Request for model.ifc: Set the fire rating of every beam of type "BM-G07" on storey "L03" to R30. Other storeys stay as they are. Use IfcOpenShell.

First a look at what the model holds.

```python
import ifcopenshell
import ifcopenshell.util.element

model = ifcopenshell.open("model.ifc")
print(model.schema)
storey = next(s for s in model.by_type("IfcBuildingStorey") if s.Name == "L03")
beams = [e for e in ifcopenshell.util.element.get_decomposition(storey) if e.is_a("IfcBeam")]
seen = {}
for e in beams:
    element_type = ifcopenshell.util.element.get_type(e)
    key = (element_type.Name if element_type != e and element_type else None, ifcopenshell.util.element.get_pset(e, "Pset_BeamCommon", "FireRating"))
    seen[key] = seen.get(key, 0) + 1
for (name, value), count in sorted(seen.items(), key=str):
    print(count, "x", name, "|", value)
```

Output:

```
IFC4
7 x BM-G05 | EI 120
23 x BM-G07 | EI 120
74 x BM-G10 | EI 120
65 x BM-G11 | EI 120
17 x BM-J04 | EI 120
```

```python
import ifcopenshell
import ifcopenshell.api.pset
import ifcopenshell.util.element

model = ifcopenshell.open("model.ifc")

storey = next(s for s in model.by_type("IfcBuildingStorey") if s.Name == "L03")
beams = [e for e in ifcopenshell.util.element.get_decomposition(storey) if e.is_a("IfcBeam")]

count = 0
for e in beams:
    element_type = ifcopenshell.util.element.get_type(e)
    if element_type in (None, e) or element_type.Name != "BM-G07":
        continue
    # add_pset returns the element's existing set when there is one.
    pset = ifcopenshell.api.pset.add_pset(model, product=e, name="Pset_BeamCommon")
    ifcopenshell.api.pset.edit_pset(model, pset=pset, properties={"FireRating": "R30"})
    count += 1

print(count, "beams updated")

model.write("model_edited.ifc")
```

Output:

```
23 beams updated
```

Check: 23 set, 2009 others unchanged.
